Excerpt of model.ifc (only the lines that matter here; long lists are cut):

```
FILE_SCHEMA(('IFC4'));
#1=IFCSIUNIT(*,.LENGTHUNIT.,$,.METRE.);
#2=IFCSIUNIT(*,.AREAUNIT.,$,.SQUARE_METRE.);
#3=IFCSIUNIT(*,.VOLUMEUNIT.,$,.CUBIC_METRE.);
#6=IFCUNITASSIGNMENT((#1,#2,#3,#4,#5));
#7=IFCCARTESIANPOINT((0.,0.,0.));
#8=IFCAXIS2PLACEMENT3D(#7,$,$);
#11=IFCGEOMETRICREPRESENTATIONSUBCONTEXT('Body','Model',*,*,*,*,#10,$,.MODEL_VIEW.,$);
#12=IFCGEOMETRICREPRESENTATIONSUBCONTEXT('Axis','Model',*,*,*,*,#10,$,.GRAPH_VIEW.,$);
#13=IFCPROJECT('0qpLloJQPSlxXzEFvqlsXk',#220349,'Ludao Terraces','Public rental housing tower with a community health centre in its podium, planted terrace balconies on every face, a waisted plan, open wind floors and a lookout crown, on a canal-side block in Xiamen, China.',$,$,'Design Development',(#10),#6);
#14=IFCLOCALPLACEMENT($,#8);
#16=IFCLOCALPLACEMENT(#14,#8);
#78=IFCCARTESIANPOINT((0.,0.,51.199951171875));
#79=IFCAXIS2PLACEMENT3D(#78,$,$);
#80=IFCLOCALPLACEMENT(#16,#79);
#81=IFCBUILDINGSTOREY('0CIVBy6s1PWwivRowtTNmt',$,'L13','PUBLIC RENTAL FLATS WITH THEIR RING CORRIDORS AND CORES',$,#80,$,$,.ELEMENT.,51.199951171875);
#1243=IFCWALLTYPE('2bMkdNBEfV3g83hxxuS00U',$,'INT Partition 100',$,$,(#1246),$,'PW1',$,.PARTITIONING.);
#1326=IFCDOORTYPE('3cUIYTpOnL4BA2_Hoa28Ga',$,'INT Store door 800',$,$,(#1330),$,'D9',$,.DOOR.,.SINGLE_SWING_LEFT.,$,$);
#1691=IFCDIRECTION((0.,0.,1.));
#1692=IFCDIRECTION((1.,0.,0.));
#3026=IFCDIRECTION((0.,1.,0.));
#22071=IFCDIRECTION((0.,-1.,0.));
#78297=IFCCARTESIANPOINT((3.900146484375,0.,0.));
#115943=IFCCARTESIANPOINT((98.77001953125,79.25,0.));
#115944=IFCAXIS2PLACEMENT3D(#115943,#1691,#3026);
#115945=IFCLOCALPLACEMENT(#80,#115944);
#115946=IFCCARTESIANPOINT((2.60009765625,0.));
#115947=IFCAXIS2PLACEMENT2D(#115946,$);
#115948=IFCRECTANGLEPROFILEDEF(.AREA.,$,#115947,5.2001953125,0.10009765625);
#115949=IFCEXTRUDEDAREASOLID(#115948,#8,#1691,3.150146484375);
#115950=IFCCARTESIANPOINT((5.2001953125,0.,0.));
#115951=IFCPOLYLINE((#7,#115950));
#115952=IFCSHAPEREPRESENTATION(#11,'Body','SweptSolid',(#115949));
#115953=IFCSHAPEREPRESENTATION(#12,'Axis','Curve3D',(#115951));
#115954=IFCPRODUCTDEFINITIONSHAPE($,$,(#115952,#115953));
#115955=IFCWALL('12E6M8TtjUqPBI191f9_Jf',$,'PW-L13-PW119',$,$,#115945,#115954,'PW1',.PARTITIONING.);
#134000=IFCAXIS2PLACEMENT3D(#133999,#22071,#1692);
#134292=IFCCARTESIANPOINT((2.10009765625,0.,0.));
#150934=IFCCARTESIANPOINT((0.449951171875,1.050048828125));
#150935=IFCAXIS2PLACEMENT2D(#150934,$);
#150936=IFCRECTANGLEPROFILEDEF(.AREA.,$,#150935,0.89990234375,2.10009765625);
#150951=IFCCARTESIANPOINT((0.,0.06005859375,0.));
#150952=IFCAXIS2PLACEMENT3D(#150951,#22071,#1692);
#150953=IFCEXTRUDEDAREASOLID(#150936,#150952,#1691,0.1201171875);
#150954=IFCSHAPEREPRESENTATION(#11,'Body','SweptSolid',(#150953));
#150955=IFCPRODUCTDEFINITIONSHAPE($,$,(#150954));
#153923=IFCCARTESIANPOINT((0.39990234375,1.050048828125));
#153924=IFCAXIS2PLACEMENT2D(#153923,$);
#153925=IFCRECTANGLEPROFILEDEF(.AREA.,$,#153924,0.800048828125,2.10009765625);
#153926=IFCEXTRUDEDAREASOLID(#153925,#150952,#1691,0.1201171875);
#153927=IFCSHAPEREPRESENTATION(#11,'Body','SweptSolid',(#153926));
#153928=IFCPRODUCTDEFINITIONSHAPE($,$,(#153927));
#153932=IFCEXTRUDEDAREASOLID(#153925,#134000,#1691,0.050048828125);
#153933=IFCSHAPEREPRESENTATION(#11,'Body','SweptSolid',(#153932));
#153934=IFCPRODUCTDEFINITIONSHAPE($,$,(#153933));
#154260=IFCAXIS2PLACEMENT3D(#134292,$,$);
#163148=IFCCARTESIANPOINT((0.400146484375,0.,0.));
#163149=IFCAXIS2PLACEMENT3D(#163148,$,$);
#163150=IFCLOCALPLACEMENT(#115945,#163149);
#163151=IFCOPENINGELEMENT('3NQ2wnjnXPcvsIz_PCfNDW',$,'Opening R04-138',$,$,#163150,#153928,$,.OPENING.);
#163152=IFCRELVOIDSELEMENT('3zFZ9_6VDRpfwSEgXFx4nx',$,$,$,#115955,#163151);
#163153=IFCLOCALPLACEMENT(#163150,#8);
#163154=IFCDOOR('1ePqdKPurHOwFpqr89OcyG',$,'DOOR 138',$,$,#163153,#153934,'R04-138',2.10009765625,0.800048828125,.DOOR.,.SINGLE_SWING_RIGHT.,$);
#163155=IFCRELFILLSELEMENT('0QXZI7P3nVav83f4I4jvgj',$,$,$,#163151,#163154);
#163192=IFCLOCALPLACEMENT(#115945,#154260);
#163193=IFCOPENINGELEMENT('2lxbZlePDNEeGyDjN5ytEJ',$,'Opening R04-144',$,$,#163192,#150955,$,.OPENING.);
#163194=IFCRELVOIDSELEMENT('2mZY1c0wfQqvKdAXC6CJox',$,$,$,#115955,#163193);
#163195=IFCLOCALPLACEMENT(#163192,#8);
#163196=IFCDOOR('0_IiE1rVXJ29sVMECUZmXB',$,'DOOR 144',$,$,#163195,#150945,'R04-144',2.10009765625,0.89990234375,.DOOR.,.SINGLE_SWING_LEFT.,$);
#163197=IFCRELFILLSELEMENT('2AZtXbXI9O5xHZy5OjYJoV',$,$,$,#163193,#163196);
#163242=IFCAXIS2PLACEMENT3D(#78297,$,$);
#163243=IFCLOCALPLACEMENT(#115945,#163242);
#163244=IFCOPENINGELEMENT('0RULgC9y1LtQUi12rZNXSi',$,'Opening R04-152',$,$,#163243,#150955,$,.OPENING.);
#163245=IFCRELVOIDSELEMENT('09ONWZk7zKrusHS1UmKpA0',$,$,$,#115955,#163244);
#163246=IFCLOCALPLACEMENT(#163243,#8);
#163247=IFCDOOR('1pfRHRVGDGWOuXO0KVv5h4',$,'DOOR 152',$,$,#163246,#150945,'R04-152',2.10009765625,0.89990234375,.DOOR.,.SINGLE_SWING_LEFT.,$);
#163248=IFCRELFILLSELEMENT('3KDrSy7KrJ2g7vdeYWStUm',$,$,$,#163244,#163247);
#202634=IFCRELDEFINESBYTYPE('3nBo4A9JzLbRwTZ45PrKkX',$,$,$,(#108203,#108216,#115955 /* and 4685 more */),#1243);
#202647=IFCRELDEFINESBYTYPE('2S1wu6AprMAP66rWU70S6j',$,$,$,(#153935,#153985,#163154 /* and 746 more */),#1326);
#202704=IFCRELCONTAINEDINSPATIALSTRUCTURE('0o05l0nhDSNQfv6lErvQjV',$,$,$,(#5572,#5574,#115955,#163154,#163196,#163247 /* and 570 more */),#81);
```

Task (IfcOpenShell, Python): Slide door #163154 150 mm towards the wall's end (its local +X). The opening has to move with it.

```python
import ifcopenshell
import ifcopenshell.api.geometry
import ifcopenshell.util.placement

model = ifcopenshell.open("model.ifc")

door = model.by_guid("1ePqdKPurHOwFpqr89OcyG")
opening = door.FillsVoids[0].RelatingOpeningElement
wall = opening.VoidsElements[0].RelatingBuildingElement

wall_matrix = ifcopenshell.util.placement.get_local_placement(wall.ObjectPlacement)
shift = wall_matrix[:3, 0] * 0.15
before = ifcopenshell.util.placement.get_local_placement(door.ObjectPlacement)[:3, 3].copy()

# The door is placed relative to its opening, so it follows when the opening moves.
matrix = ifcopenshell.util.placement.get_local_placement(opening.ObjectPlacement)
matrix[:3, 3] += shift
ifcopenshell.api.geometry.edit_object_placement(
    model, product=opening, matrix=matrix, is_si=False, should_transform_children=True
)

after = ifcopenshell.util.placement.get_local_placement(door.ObjectPlacement)[:3, 3]
print("door moved by", (after - before).round(3) + 0.0)

model.write("model_updated.ifc")
```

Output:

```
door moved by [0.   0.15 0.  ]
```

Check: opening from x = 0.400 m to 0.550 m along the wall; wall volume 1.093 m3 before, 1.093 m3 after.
